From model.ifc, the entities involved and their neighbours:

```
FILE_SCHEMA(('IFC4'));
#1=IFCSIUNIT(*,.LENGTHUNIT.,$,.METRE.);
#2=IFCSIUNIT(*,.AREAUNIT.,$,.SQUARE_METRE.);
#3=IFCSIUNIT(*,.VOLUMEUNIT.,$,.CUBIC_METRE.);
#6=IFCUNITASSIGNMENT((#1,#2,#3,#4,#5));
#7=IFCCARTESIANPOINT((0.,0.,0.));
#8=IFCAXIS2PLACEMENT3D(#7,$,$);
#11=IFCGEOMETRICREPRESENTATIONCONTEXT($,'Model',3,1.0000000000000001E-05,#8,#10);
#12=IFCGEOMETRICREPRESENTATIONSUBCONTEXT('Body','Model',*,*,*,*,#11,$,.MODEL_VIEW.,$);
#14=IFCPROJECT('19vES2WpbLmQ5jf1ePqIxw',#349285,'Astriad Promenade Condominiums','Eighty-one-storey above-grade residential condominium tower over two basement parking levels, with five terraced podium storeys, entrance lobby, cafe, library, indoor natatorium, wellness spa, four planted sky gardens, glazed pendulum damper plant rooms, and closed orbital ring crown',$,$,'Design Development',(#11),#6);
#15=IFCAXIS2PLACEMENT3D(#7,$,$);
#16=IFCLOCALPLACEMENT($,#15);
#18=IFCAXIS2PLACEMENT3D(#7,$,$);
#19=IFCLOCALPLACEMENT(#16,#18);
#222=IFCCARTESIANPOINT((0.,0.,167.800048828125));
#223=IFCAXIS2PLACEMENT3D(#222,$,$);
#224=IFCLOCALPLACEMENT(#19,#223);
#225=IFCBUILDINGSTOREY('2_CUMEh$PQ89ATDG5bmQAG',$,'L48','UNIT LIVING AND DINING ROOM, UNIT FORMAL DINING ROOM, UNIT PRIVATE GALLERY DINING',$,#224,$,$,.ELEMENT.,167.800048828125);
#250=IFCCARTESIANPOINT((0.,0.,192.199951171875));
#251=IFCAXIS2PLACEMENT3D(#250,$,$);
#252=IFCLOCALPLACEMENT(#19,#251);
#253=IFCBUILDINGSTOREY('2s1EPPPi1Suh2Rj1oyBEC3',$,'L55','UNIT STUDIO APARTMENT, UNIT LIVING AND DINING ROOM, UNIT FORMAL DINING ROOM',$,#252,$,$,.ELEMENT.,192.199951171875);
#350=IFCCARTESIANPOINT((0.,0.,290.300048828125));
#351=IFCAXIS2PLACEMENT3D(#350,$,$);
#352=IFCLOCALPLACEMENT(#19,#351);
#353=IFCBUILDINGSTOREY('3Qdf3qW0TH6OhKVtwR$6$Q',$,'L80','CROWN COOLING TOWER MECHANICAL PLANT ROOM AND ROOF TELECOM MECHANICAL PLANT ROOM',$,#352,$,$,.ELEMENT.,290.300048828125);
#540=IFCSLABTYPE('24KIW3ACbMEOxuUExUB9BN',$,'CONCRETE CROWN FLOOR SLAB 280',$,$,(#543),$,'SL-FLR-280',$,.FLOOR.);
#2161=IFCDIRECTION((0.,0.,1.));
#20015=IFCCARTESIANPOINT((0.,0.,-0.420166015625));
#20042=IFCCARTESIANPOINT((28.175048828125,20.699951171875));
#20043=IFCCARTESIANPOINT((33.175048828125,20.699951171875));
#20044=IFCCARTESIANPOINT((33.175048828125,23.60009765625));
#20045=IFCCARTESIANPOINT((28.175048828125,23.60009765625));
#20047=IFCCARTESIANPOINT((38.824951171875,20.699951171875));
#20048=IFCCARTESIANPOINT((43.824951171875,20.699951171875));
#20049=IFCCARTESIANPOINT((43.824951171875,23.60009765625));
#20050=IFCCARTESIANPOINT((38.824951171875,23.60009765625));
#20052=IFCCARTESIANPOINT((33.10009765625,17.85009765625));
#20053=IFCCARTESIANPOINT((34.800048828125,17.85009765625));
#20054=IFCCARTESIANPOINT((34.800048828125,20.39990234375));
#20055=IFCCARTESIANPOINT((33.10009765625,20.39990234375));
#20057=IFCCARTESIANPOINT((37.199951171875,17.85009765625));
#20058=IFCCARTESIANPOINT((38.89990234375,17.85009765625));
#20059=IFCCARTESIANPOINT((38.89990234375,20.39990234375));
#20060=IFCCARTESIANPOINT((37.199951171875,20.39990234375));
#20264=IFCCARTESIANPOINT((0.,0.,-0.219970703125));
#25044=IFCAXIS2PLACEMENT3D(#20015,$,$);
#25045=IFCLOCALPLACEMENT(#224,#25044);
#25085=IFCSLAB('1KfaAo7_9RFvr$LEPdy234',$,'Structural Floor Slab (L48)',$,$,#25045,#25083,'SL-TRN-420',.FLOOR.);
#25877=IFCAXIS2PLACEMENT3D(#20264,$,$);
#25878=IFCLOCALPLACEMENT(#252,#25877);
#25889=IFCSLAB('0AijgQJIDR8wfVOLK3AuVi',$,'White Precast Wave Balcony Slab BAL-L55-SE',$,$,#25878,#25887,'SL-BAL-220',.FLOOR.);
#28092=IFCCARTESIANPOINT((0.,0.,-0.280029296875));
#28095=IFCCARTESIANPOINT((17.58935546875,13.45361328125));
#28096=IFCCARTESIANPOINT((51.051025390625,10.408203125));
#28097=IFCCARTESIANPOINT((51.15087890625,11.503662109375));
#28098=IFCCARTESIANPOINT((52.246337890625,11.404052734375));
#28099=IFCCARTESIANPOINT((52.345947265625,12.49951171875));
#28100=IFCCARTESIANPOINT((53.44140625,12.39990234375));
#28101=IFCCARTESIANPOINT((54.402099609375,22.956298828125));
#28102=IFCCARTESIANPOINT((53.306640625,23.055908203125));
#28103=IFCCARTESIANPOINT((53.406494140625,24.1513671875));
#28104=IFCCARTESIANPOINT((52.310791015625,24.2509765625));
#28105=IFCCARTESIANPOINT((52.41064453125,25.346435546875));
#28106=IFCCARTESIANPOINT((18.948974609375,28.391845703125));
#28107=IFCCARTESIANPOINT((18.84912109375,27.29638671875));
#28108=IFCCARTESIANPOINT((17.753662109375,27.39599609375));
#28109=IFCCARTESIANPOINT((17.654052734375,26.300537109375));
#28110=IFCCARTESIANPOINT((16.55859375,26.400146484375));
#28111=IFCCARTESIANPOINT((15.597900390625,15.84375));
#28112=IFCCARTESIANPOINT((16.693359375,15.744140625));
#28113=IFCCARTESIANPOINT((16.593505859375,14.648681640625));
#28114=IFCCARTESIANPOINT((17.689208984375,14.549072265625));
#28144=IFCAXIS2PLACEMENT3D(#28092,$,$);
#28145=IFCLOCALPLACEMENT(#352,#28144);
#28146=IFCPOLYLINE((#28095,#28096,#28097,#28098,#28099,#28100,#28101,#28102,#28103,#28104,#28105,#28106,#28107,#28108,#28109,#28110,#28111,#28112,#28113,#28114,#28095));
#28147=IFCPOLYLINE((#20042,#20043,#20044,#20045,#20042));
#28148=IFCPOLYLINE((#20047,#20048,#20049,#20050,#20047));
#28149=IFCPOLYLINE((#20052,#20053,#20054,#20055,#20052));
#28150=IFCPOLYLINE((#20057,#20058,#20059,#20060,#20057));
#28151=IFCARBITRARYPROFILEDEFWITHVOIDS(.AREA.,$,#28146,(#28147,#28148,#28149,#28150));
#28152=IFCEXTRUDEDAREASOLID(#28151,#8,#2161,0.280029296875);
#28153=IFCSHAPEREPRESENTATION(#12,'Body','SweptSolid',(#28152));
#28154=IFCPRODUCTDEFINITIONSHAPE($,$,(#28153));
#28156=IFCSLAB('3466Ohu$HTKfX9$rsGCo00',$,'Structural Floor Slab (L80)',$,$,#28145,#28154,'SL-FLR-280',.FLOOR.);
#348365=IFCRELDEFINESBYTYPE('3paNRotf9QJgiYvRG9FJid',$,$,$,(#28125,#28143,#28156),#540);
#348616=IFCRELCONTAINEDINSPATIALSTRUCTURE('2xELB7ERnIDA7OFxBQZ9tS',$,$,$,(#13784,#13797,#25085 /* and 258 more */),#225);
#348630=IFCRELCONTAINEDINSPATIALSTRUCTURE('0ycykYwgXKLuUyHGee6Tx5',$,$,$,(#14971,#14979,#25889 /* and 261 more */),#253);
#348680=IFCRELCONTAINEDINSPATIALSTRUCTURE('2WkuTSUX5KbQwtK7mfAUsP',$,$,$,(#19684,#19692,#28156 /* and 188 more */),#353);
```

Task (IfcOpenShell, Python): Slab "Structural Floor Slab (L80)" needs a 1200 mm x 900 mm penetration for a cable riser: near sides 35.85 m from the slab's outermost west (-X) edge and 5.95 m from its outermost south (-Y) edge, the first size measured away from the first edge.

```python
import numpy as np
import ifcopenshell
import ifcopenshell.api.feature
import ifcopenshell.api.geometry
import ifcopenshell.api.root
import ifcopenshell.geom
import ifcopenshell.util.placement
import ifcopenshell.util.representation
import ifcopenshell.util.shape
import ifcopenshell.util.unit

model = ifcopenshell.open("model.ifc")
unit_scale = ifcopenshell.util.unit.calculate_unit_scale(model)
settings = ifcopenshell.geom.settings()


def volume(element):
    """Net volume in cubic metres, openings subtracted."""
    shape = ifcopenshell.geom.create_shape(settings, element)
    return ifcopenshell.util.shape.get_volume(shape.geometry)


slab = model.by_guid("3466Ohu$HTKfX9$rsGCo00")
before = volume(slab)

# Extent in the slab's own axes, in metres. The edges named are its -X and -Y sides.
slab_shape = ifcopenshell.geom.create_shape(settings, slab)
vertices = ifcopenshell.util.shape.get_vertices(slab_shape.geometry)
x_min, y_min, bottom = vertices.min(axis=0)
top = vertices[:, 2].max()

opening = ifcopenshell.api.root.create_entity(model, ifc_class="IfcOpeningElement", name="Cable riser opening", predefined_type="OPENING")
context = ifcopenshell.util.representation.get_context(model, "Model", "Body", "MODEL_VIEW")
width, depth = 1.2, 0.9
outline = [(0.0, 0.0), (width, 0.0), (width, depth), (0.0, depth), (0.0, 0.0)]
# Overshoot both faces by 50 mm so the cut is clean.
shape = ifcopenshell.api.geometry.add_slab_representation(
    model, context=context, depth=top - bottom + 0.1, polyline=outline
)
ifcopenshell.api.geometry.assign_representation(model, product=opening, representation=shape)

matrix = ifcopenshell.util.placement.get_local_placement(slab.ObjectPlacement)
matrix[:, 3] = matrix @ np.append(np.array([x_min + 35.85, y_min + 5.95, bottom - 0.05]) / unit_scale, 1.0)
ifcopenshell.api.geometry.edit_object_placement(model, product=opening, matrix=matrix, is_si=False)
ifcopenshell.api.feature.add_feature(model, feature=opening, element=slab)

after = volume(slab)

print(f"slab volume {before:.3f} -> {after:.3f} m3")

model.write("model_updated.ifc")
```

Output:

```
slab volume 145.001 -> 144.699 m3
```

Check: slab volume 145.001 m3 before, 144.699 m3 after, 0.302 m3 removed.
